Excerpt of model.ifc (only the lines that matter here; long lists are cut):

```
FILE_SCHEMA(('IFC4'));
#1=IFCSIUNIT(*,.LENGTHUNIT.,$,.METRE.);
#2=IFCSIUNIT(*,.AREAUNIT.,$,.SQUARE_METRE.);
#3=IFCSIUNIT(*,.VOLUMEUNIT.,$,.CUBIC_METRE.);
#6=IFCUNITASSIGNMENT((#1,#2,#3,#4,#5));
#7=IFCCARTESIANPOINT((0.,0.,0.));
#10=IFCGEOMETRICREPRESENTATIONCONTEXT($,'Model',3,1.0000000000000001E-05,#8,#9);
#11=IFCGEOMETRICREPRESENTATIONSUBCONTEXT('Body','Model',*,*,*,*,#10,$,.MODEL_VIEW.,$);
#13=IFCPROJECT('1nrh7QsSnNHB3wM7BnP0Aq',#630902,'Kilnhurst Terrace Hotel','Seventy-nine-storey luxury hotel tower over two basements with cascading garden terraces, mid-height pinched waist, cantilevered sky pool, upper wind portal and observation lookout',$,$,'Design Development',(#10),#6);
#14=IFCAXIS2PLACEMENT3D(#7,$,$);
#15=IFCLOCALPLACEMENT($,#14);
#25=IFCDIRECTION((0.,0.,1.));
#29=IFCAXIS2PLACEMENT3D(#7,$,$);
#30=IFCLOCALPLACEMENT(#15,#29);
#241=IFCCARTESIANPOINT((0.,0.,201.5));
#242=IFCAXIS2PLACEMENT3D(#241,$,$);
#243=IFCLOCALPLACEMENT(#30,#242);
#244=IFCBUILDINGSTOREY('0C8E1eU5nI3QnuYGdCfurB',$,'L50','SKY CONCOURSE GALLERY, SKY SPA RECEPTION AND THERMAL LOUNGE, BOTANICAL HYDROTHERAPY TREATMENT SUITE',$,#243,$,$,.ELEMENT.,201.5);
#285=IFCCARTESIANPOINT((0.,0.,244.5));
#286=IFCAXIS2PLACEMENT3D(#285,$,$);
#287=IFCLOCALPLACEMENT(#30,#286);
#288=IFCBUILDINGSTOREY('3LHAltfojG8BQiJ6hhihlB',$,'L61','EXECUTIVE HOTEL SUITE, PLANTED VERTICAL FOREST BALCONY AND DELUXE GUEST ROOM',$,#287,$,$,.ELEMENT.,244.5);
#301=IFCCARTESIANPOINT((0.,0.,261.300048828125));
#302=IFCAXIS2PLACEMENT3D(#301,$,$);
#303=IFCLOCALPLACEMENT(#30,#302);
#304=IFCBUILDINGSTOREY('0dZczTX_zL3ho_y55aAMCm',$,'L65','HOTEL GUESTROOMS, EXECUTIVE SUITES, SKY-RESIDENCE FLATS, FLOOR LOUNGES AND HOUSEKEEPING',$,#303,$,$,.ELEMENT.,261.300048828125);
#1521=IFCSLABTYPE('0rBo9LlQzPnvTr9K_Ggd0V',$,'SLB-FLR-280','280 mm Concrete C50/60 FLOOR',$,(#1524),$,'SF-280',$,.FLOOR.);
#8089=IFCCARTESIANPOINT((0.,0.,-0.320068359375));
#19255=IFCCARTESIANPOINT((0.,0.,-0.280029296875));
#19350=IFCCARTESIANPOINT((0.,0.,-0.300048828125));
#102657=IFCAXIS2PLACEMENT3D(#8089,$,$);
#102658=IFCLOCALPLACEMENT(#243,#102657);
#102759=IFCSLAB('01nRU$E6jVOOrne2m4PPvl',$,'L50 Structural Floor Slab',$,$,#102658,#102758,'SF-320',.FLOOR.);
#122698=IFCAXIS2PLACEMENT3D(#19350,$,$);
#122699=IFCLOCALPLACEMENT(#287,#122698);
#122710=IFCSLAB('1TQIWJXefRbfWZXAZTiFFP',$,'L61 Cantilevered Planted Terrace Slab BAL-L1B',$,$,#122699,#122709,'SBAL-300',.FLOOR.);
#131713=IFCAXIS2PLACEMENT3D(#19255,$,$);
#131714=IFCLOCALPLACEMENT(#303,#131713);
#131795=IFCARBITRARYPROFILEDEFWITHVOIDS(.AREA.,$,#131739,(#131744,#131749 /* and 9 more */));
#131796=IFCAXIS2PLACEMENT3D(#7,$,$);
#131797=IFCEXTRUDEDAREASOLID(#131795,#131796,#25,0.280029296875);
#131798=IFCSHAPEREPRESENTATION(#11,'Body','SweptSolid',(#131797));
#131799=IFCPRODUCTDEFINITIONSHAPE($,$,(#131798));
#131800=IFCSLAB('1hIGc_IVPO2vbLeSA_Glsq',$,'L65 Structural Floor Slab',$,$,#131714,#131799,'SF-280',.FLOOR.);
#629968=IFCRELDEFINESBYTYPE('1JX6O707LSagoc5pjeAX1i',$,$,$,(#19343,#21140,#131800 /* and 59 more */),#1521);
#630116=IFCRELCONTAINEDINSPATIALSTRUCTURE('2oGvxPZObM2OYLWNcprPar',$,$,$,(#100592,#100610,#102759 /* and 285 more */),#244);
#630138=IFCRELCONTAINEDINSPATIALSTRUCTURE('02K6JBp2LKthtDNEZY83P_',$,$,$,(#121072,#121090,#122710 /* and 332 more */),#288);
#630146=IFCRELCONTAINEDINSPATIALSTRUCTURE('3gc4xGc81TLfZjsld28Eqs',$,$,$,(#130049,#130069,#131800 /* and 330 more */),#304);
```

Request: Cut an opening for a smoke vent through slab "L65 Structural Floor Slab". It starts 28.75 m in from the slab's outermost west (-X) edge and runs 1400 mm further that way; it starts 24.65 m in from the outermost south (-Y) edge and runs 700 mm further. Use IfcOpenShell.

```python
import numpy as np
import ifcopenshell
import ifcopenshell.api.feature
import ifcopenshell.api.geometry
import ifcopenshell.api.root
import ifcopenshell.geom
import ifcopenshell.util.placement
import ifcopenshell.util.representation
import ifcopenshell.util.shape
import ifcopenshell.util.unit

model = ifcopenshell.open("model.ifc")
unit_scale = ifcopenshell.util.unit.calculate_unit_scale(model)
settings = ifcopenshell.geom.settings()


def volume(element):
    """Net volume in cubic metres, openings subtracted."""
    shape = ifcopenshell.geom.create_shape(settings, element)
    return ifcopenshell.util.shape.get_volume(shape.geometry)


slab = model.by_id(131800)
before = volume(slab)

# Extent in the slab's own axes, in metres. The edges named are its -X and -Y sides.
slab_shape = ifcopenshell.geom.create_shape(settings, slab)
vertices = ifcopenshell.util.shape.get_vertices(slab_shape.geometry)
x_min, y_min, bottom = vertices.min(axis=0)
top = vertices[:, 2].max()

opening = ifcopenshell.api.root.create_entity(model, ifc_class="IfcOpeningElement", name="Smoke vent opening", predefined_type="OPENING")
context = ifcopenshell.util.representation.get_context(model, "Model", "Body", "MODEL_VIEW")
width, depth = 1.4, 0.7
outline = [(0.0, 0.0), (width, 0.0), (width, depth), (0.0, depth), (0.0, 0.0)]
# Overshoot both faces by 50 mm so the cut is clean.
shape = ifcopenshell.api.geometry.add_slab_representation(
    model, context=context, depth=top - bottom + 0.1, polyline=outline
)
ifcopenshell.api.geometry.assign_representation(model, product=opening, representation=shape)

matrix = ifcopenshell.util.placement.get_local_placement(slab.ObjectPlacement)
matrix[:, 3] = matrix @ np.append(np.array([x_min + 28.75, y_min + 24.65, bottom - 0.05]) / unit_scale, 1.0)
ifcopenshell.api.geometry.edit_object_placement(model, product=opening, matrix=matrix, is_si=False)
ifcopenshell.api.feature.add_feature(model, feature=opening, element=slab)

after = volume(slab)

print(f"slab volume {before:.3f} -> {after:.3f} m3")

model.write("model_v2.ifc")
```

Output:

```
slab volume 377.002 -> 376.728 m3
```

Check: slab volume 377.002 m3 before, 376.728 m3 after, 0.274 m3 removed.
